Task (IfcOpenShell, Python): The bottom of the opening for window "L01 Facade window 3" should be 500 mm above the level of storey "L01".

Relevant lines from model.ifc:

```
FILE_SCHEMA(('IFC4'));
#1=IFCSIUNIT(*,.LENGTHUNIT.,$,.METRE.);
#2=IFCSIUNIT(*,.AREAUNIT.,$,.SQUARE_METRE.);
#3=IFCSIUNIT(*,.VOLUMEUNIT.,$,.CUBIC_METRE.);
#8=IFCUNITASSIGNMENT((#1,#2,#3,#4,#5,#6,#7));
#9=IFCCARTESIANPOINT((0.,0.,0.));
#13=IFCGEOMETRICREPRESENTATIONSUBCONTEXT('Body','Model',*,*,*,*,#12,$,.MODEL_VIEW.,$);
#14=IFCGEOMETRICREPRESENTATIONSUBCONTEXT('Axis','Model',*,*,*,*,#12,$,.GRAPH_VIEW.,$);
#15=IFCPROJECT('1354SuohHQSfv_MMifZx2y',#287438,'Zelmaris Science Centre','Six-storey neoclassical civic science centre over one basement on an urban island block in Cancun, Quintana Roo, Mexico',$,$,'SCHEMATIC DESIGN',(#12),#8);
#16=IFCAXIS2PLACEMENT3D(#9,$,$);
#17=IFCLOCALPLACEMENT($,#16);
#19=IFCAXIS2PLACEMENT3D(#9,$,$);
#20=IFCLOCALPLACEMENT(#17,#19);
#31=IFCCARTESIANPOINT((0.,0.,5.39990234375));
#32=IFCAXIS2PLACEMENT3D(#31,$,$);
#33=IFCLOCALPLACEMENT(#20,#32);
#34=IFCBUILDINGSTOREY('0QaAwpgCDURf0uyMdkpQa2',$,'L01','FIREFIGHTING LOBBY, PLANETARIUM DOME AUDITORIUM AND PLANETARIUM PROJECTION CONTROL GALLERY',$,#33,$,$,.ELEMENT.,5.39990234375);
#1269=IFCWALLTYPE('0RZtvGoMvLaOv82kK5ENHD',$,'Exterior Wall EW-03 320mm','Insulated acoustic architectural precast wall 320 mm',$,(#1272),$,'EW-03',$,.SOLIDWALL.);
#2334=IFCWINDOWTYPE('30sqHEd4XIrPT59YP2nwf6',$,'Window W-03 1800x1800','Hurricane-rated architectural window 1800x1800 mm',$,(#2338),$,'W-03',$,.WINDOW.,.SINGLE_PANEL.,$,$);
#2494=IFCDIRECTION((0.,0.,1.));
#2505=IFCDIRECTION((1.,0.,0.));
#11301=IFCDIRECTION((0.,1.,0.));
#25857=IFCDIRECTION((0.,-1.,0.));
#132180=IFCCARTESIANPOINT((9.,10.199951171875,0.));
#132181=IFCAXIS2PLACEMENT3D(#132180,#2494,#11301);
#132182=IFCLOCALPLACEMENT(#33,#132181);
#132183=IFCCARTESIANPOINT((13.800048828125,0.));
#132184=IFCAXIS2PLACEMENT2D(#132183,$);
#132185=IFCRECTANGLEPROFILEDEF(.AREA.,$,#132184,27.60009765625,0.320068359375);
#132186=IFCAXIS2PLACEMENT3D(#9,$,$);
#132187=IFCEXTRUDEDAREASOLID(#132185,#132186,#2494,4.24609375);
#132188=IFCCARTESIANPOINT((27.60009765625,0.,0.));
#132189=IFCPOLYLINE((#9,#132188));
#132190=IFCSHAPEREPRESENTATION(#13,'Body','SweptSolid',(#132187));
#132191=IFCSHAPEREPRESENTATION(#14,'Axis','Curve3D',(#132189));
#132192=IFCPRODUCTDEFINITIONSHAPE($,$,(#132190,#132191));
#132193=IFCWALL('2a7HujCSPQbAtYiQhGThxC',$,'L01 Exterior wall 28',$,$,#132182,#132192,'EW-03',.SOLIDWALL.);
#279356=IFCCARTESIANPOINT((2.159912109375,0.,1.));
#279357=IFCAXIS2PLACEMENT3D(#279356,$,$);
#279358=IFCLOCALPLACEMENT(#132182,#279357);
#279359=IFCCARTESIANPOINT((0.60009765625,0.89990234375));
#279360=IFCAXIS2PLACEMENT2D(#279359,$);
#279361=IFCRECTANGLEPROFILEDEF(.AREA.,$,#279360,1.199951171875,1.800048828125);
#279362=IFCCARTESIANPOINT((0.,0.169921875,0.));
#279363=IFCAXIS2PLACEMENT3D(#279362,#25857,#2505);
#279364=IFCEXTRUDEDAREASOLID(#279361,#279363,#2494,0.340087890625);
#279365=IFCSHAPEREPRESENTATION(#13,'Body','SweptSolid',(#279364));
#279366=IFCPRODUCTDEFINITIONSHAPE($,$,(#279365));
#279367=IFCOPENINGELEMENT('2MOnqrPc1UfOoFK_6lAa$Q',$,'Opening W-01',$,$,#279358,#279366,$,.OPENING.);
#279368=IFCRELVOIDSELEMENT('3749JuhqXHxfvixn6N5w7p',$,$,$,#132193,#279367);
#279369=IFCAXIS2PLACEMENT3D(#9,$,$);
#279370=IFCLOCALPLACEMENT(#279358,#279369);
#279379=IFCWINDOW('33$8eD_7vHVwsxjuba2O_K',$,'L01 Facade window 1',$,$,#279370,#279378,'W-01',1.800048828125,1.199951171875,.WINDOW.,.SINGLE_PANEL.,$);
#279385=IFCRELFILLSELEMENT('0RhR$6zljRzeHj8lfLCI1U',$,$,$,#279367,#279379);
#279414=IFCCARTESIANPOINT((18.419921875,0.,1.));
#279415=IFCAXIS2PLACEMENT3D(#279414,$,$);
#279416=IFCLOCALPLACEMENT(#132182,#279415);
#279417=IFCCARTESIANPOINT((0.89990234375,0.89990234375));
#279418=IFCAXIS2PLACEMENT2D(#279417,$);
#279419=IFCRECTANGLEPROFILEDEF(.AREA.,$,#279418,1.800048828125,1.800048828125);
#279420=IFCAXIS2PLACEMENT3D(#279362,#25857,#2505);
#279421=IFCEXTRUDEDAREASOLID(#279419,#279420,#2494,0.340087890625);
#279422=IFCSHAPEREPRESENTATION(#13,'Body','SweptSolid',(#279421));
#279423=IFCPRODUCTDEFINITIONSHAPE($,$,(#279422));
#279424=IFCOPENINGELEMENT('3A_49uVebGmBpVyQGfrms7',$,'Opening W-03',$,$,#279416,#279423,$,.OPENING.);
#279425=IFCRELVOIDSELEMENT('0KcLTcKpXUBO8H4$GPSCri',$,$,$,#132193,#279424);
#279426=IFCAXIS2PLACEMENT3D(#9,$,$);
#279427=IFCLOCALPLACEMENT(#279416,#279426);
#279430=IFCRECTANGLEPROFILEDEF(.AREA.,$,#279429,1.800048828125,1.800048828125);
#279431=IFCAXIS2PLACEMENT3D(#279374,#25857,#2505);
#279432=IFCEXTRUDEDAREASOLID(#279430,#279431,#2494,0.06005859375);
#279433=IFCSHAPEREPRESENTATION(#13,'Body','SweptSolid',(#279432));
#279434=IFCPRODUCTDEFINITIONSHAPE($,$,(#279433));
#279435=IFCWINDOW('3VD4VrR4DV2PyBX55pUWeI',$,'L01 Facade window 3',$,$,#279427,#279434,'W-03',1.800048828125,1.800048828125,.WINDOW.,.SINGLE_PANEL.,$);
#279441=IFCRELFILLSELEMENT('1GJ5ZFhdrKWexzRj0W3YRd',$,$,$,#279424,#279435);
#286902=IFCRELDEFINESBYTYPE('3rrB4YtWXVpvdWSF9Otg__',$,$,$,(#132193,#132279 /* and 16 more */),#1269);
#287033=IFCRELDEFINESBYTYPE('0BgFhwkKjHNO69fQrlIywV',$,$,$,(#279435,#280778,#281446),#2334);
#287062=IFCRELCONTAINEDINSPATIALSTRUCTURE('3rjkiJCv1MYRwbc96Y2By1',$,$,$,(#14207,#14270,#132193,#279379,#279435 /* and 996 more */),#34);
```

```python
import numpy as np
import ifcopenshell
import ifcopenshell.api.geometry
import ifcopenshell.geom
import ifcopenshell.util.element
import ifcopenshell.util.placement
import ifcopenshell.util.shape
import ifcopenshell.util.unit

model = ifcopenshell.open("model.ifc")
unit_scale = ifcopenshell.util.unit.calculate_unit_scale(model)

window = model.by_guid("3VD4VrR4DV2PyBX55pUWeI")
opening = window.FillsVoids[0].RelatingOpeningElement
storey = ifcopenshell.util.element.get_container(window, ifc_class="IfcBuildingStorey")
level = ifcopenshell.util.placement.get_local_placement(storey.ObjectPlacement)[2, 3]

# The opening's origin need not be at the sill, so measure its lowest point.
shape = ifcopenshell.geom.create_shape(ifcopenshell.geom.settings(), opening)
bottom = ifcopenshell.util.shape.get_shape_bottom_elevation(shape, shape.geometry) / unit_scale
dz = level + 0.5 - bottom

shift = np.array([0.0, 0.0, dz])
# The window is placed relative to its opening, so it follows when the opening moves.
matrix = ifcopenshell.util.placement.get_local_placement(opening.ObjectPlacement)
matrix[:3, 3] += shift
ifcopenshell.api.geometry.edit_object_placement(
    model, product=opening, matrix=matrix, is_si=False, should_transform_children=True
)

print(f"moved by {dz * unit_scale:+.3f} m")

model.write("model-out.ifc")
```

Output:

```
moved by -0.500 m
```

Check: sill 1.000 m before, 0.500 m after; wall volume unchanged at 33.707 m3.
